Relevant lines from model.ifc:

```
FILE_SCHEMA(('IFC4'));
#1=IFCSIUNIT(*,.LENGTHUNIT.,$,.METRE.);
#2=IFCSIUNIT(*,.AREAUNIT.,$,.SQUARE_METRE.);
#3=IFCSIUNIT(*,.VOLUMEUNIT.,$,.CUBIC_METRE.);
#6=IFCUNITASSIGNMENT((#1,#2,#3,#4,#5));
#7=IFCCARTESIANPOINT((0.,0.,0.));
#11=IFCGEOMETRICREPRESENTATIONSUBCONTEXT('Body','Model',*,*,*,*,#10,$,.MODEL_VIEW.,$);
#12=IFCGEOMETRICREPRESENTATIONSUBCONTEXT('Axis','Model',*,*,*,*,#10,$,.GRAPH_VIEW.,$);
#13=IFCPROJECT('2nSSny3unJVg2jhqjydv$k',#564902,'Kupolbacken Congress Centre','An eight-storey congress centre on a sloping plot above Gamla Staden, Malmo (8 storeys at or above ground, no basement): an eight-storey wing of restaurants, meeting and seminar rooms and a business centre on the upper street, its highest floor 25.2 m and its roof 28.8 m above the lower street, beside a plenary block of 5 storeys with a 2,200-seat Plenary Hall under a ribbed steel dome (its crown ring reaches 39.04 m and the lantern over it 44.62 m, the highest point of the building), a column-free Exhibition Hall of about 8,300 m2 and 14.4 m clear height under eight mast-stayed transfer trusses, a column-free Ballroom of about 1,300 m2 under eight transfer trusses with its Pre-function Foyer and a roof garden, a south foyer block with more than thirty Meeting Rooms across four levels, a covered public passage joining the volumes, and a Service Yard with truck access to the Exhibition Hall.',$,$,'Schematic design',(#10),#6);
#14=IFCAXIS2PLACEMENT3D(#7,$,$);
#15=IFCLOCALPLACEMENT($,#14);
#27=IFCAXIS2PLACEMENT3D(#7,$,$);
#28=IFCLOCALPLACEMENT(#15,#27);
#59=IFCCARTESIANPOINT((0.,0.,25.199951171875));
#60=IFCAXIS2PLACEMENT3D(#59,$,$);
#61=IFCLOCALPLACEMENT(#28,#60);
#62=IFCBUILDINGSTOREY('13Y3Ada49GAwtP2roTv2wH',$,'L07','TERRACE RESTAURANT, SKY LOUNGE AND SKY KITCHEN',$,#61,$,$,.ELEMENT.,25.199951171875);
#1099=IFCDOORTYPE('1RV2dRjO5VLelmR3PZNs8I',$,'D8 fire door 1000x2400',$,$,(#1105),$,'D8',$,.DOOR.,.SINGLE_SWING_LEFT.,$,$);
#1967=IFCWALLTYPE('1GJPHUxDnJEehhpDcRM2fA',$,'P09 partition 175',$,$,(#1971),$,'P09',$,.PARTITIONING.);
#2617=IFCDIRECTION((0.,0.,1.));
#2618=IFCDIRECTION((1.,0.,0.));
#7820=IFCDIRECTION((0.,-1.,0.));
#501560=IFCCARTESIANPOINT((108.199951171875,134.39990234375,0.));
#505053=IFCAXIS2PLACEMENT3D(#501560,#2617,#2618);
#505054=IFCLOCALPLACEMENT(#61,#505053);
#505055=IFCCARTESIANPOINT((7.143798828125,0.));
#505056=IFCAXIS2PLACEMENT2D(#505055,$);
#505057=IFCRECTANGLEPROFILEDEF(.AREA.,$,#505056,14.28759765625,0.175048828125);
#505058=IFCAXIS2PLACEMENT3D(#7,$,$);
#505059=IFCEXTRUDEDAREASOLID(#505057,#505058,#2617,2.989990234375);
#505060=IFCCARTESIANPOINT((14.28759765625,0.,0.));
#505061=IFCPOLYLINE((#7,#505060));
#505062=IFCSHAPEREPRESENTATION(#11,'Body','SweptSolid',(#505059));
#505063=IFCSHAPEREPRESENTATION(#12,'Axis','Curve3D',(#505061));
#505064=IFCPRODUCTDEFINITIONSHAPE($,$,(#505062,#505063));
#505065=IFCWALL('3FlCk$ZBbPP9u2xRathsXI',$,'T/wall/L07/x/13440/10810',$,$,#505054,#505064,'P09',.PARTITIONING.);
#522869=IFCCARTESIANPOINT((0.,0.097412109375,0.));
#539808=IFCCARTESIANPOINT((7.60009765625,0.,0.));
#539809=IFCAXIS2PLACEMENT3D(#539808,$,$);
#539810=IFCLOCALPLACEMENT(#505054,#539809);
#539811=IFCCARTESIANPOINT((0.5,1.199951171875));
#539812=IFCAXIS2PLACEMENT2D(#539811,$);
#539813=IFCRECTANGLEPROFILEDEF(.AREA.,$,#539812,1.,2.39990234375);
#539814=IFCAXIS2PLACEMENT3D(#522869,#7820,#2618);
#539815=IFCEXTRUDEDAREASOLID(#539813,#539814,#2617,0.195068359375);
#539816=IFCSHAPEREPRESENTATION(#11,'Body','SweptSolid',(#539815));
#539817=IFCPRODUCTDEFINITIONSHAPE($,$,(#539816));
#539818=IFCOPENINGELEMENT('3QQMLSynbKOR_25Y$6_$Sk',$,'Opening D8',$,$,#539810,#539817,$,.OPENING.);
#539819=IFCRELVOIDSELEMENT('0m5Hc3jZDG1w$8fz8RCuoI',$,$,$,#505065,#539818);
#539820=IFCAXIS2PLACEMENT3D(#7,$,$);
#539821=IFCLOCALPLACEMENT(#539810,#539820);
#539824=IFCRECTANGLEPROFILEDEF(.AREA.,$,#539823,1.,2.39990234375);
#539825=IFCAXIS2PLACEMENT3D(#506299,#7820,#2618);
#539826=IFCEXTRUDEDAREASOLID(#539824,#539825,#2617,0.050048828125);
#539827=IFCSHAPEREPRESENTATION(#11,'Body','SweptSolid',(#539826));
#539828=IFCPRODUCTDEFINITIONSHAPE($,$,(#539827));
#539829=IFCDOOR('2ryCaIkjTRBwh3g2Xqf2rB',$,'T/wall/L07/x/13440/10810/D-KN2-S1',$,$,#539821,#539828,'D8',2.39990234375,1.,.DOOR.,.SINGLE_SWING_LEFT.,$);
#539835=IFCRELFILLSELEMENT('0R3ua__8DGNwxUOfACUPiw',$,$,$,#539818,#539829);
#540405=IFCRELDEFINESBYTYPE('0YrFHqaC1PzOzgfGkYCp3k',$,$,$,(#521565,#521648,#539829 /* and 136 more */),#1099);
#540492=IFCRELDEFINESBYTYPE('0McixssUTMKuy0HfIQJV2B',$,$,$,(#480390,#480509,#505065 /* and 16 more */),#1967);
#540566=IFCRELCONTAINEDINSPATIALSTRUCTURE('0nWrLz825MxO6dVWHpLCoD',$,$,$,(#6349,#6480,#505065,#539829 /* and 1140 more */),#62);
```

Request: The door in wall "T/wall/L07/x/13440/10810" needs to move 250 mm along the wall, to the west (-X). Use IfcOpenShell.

```python
import ifcopenshell
import ifcopenshell.api.geometry
import ifcopenshell.util.placement

model = ifcopenshell.open("model.ifc")

door = model.by_guid("2ryCaIkjTRBwh3g2Xqf2rB")
opening = door.FillsVoids[0].RelatingOpeningElement
wall = opening.VoidsElements[0].RelatingBuildingElement

wall_matrix = ifcopenshell.util.placement.get_local_placement(wall.ObjectPlacement)
shift = wall_matrix[:3, 0] * -0.25
before = ifcopenshell.util.placement.get_local_placement(door.ObjectPlacement)[:3, 3].copy()

# The door is placed relative to its opening, so it follows when the opening moves.
matrix = ifcopenshell.util.placement.get_local_placement(opening.ObjectPlacement)
matrix[:3, 3] += shift
ifcopenshell.api.geometry.edit_object_placement(
    model, product=opening, matrix=matrix, is_si=False, should_transform_children=True
)

after = ifcopenshell.util.placement.get_local_placement(door.ObjectPlacement)[:3, 3]
print("door moved by", (after - before).round(3) + 0.0)

model.write("model_updated.ifc")
```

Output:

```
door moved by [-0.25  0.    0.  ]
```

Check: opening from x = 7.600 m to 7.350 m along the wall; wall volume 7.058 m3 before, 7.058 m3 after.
